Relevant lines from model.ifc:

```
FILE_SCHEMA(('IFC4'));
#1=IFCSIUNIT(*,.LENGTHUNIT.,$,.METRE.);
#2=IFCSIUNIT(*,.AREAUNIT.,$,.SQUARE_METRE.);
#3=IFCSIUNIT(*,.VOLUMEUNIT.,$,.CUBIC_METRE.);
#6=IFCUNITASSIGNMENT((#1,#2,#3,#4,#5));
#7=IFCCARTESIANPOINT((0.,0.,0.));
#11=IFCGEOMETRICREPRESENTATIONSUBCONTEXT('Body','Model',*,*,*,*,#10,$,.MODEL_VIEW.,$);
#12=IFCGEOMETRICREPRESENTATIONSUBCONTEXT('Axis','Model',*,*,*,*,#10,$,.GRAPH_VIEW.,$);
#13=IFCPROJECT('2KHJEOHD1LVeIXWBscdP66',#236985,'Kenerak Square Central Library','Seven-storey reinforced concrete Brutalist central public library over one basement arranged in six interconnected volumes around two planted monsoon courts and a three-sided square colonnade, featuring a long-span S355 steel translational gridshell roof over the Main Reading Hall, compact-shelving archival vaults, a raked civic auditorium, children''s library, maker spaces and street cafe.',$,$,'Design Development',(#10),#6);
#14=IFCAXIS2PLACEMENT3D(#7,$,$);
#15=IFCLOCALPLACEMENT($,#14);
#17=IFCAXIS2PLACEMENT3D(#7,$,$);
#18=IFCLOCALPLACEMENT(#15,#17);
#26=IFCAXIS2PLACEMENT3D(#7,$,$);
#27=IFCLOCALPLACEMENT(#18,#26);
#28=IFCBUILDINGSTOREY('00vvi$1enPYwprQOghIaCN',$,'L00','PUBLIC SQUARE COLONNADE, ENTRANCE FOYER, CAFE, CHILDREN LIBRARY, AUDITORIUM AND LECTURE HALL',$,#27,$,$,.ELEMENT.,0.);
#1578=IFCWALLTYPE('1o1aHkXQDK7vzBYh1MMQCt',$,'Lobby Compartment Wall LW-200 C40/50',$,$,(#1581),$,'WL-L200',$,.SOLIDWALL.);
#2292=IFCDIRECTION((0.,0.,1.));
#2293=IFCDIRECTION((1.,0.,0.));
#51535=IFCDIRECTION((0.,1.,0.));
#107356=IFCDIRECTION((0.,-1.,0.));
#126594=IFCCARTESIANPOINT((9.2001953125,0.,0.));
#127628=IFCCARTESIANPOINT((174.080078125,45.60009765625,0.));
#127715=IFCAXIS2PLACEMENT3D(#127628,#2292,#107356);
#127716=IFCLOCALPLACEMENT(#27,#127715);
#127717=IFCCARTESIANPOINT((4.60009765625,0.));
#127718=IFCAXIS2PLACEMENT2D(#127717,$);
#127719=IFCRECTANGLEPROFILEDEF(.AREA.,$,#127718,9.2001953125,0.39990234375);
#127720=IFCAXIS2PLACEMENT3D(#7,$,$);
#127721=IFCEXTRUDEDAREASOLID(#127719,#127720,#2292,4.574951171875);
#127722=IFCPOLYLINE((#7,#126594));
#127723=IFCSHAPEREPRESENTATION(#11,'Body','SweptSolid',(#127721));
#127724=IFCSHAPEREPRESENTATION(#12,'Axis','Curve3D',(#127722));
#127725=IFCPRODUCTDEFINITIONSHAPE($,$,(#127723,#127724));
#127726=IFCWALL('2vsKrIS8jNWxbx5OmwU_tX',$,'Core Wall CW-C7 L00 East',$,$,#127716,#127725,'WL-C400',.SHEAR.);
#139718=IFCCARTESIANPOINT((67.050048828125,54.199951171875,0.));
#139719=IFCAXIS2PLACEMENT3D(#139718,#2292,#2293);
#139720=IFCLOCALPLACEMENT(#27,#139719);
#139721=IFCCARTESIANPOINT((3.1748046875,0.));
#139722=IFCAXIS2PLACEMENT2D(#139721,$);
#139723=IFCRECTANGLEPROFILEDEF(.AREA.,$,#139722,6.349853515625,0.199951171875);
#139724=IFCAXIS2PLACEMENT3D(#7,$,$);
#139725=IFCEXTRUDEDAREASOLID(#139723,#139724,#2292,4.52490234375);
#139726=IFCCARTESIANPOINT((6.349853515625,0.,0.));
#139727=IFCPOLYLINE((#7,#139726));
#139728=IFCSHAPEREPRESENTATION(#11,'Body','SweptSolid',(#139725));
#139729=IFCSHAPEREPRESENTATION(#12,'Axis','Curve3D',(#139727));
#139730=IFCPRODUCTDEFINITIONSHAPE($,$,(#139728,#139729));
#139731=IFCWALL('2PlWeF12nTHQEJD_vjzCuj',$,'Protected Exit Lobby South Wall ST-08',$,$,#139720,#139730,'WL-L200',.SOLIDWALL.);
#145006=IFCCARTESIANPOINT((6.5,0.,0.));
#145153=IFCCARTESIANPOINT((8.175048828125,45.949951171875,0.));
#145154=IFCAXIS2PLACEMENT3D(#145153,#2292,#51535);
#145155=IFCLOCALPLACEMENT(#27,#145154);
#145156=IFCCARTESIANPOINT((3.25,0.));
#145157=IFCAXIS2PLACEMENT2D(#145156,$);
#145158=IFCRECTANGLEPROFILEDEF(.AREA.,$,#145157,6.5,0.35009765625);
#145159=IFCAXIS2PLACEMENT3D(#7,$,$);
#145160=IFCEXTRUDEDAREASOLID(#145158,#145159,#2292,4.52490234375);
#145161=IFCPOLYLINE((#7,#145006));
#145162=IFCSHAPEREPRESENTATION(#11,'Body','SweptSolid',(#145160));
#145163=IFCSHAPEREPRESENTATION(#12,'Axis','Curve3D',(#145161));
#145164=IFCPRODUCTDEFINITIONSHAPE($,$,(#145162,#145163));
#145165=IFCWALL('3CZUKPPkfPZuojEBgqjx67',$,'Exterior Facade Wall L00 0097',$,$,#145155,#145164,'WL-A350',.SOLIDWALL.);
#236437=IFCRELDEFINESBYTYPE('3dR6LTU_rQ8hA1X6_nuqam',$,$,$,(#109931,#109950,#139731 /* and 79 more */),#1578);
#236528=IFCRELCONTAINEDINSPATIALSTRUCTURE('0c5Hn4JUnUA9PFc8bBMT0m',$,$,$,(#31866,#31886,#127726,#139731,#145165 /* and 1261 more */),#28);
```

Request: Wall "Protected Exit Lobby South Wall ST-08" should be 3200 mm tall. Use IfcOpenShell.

```python
import ifcopenshell
import ifcopenshell.geom
import ifcopenshell.util.representation
import ifcopenshell.util.shape
import ifcopenshell.util.unit

model = ifcopenshell.open("model.ifc")
unit_scale = ifcopenshell.util.unit.calculate_unit_scale(model)
settings = ifcopenshell.geom.settings()


def volume(element):
    """Net volume in cubic metres, openings subtracted."""
    shape = ifcopenshell.geom.create_shape(settings, element)
    return ifcopenshell.util.shape.get_volume(shape.geometry)


wall = model.by_guid("2PlWeF12nTHQEJD_vjzCuj")
before = volume(wall)

body = ifcopenshell.util.representation.get_representation(wall, "Model", "Body")
solid = body.Items[0]
old_height = solid.Depth
solid.Depth = 3.2 / unit_scale
after = volume(wall)

print(f"height {old_height:g} -> {solid.Depth:g}, volume {before:.3f} -> {after:.3f} m3")

model.write("model_updated.ifc")
```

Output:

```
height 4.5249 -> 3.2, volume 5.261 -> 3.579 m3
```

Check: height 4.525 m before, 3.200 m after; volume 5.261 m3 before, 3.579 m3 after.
